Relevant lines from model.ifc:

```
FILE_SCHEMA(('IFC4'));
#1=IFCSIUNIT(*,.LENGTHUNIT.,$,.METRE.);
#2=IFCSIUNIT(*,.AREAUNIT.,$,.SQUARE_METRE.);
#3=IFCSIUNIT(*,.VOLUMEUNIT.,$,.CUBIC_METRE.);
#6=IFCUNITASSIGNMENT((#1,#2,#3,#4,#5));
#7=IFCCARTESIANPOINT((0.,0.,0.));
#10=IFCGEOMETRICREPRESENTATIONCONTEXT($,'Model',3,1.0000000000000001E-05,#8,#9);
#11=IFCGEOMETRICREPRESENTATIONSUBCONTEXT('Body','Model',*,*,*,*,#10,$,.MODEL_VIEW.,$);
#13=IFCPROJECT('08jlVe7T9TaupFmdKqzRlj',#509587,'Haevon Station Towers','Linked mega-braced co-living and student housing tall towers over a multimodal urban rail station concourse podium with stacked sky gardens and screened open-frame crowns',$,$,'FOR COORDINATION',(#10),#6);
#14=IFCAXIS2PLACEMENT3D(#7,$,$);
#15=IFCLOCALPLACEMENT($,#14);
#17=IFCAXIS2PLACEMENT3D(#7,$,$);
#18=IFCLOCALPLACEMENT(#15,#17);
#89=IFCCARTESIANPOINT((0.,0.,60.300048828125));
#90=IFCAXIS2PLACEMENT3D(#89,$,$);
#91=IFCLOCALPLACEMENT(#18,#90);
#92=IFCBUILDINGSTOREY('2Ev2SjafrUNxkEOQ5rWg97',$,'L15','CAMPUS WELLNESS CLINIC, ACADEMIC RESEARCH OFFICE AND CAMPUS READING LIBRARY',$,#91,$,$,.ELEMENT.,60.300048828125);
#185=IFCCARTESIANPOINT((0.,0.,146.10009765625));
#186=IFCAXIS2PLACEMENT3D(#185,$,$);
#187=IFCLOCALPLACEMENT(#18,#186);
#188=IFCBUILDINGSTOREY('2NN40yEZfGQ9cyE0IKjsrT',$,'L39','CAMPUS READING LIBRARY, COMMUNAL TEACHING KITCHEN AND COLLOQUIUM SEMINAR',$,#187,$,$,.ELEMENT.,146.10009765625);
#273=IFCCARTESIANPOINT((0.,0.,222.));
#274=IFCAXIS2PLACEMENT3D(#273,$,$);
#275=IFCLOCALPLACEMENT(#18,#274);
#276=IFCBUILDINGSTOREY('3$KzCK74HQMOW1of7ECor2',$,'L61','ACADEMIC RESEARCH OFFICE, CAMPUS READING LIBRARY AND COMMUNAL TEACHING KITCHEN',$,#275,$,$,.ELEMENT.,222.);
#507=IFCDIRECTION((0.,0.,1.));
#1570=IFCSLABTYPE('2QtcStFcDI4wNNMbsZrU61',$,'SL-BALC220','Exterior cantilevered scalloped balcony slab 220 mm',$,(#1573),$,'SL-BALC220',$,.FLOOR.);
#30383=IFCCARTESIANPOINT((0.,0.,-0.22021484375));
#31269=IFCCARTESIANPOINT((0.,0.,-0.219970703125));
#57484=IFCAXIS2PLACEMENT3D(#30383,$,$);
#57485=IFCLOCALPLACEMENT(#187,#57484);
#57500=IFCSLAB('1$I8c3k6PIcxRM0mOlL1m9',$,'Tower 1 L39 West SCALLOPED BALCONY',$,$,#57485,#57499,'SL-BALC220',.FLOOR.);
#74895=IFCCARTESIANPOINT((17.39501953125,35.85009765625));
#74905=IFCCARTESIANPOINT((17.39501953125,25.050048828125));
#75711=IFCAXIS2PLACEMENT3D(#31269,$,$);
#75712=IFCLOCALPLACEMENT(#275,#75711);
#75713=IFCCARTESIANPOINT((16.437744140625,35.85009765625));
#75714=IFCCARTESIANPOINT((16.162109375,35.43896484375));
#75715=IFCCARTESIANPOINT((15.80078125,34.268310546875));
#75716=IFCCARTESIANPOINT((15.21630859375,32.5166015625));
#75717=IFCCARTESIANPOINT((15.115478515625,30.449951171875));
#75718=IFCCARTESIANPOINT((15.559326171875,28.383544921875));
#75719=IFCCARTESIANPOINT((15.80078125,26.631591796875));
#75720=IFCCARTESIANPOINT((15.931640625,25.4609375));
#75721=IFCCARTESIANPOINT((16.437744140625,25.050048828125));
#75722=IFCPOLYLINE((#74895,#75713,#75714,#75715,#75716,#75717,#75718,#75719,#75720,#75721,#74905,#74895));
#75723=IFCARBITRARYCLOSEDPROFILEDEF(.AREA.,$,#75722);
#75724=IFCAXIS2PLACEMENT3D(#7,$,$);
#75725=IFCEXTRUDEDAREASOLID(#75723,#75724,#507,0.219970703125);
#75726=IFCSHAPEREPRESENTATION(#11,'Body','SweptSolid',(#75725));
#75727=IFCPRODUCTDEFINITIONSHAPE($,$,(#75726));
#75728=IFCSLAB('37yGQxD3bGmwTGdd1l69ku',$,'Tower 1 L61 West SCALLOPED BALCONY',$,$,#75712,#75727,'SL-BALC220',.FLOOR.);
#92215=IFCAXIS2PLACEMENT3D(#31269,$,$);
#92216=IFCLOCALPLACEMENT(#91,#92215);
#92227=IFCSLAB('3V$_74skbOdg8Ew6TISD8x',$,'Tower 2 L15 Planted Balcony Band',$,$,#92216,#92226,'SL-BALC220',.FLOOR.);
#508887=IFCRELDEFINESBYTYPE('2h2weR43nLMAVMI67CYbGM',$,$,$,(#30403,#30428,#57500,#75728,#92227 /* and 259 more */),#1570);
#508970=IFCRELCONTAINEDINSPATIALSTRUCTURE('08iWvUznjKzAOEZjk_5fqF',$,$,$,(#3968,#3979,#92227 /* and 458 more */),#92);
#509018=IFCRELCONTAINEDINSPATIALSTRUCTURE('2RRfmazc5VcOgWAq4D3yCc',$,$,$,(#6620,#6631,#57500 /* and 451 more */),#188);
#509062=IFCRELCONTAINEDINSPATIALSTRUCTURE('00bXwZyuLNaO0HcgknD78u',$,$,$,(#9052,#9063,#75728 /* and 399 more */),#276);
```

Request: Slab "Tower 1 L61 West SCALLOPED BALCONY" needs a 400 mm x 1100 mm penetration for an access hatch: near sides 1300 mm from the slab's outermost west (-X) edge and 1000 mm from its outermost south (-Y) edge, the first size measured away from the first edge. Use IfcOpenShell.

```python
import numpy as np
import ifcopenshell
import ifcopenshell.api.feature
import ifcopenshell.api.geometry
import ifcopenshell.api.root
import ifcopenshell.geom
import ifcopenshell.util.placement
import ifcopenshell.util.representation
import ifcopenshell.util.shape
import ifcopenshell.util.unit

model = ifcopenshell.open("model.ifc")
unit_scale = ifcopenshell.util.unit.calculate_unit_scale(model)
settings = ifcopenshell.geom.settings()


def volume(element):
    """Net volume in cubic metres, openings subtracted."""
    shape = ifcopenshell.geom.create_shape(settings, element)
    return ifcopenshell.util.shape.get_volume(shape.geometry)


slab = model.by_guid("37yGQxD3bGmwTGdd1l69ku")
before = volume(slab)

# Extent in the slab's own axes, in metres. The edges named are its -X and -Y sides.
slab_shape = ifcopenshell.geom.create_shape(settings, slab)
vertices = ifcopenshell.util.shape.get_vertices(slab_shape.geometry)
x_min, y_min, bottom = vertices.min(axis=0)
top = vertices[:, 2].max()

opening = ifcopenshell.api.root.create_entity(model, ifc_class="IfcOpeningElement", name="Access hatch opening", predefined_type="OPENING")
context = ifcopenshell.util.representation.get_context(model, "Model", "Body", "MODEL_VIEW")
width, depth = 0.4, 1.1
outline = [(0.0, 0.0), (width, 0.0), (width, depth), (0.0, depth), (0.0, 0.0)]
# Overshoot both faces by 50 mm so the cut is clean.
shape = ifcopenshell.api.geometry.add_slab_representation(
    model, context=context, depth=top - bottom + 0.1, polyline=outline
)
ifcopenshell.api.geometry.assign_representation(model, product=opening, representation=shape)

matrix = ifcopenshell.util.placement.get_local_placement(slab.ObjectPlacement)
matrix[:, 3] = matrix @ np.append(np.array([x_min + 1.3, y_min + 1, bottom - 0.05]) / unit_scale, 1.0)
ifcopenshell.api.geometry.edit_object_placement(model, product=opening, matrix=matrix, is_si=False)
ifcopenshell.api.feature.add_feature(model, feature=opening, element=slab)

after = volume(slab)

print(f"slab volume {before:.3f} -> {after:.3f} m3")

model.write("model_edited.ifc")
```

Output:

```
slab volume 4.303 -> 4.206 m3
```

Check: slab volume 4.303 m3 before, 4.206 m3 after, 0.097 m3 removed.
